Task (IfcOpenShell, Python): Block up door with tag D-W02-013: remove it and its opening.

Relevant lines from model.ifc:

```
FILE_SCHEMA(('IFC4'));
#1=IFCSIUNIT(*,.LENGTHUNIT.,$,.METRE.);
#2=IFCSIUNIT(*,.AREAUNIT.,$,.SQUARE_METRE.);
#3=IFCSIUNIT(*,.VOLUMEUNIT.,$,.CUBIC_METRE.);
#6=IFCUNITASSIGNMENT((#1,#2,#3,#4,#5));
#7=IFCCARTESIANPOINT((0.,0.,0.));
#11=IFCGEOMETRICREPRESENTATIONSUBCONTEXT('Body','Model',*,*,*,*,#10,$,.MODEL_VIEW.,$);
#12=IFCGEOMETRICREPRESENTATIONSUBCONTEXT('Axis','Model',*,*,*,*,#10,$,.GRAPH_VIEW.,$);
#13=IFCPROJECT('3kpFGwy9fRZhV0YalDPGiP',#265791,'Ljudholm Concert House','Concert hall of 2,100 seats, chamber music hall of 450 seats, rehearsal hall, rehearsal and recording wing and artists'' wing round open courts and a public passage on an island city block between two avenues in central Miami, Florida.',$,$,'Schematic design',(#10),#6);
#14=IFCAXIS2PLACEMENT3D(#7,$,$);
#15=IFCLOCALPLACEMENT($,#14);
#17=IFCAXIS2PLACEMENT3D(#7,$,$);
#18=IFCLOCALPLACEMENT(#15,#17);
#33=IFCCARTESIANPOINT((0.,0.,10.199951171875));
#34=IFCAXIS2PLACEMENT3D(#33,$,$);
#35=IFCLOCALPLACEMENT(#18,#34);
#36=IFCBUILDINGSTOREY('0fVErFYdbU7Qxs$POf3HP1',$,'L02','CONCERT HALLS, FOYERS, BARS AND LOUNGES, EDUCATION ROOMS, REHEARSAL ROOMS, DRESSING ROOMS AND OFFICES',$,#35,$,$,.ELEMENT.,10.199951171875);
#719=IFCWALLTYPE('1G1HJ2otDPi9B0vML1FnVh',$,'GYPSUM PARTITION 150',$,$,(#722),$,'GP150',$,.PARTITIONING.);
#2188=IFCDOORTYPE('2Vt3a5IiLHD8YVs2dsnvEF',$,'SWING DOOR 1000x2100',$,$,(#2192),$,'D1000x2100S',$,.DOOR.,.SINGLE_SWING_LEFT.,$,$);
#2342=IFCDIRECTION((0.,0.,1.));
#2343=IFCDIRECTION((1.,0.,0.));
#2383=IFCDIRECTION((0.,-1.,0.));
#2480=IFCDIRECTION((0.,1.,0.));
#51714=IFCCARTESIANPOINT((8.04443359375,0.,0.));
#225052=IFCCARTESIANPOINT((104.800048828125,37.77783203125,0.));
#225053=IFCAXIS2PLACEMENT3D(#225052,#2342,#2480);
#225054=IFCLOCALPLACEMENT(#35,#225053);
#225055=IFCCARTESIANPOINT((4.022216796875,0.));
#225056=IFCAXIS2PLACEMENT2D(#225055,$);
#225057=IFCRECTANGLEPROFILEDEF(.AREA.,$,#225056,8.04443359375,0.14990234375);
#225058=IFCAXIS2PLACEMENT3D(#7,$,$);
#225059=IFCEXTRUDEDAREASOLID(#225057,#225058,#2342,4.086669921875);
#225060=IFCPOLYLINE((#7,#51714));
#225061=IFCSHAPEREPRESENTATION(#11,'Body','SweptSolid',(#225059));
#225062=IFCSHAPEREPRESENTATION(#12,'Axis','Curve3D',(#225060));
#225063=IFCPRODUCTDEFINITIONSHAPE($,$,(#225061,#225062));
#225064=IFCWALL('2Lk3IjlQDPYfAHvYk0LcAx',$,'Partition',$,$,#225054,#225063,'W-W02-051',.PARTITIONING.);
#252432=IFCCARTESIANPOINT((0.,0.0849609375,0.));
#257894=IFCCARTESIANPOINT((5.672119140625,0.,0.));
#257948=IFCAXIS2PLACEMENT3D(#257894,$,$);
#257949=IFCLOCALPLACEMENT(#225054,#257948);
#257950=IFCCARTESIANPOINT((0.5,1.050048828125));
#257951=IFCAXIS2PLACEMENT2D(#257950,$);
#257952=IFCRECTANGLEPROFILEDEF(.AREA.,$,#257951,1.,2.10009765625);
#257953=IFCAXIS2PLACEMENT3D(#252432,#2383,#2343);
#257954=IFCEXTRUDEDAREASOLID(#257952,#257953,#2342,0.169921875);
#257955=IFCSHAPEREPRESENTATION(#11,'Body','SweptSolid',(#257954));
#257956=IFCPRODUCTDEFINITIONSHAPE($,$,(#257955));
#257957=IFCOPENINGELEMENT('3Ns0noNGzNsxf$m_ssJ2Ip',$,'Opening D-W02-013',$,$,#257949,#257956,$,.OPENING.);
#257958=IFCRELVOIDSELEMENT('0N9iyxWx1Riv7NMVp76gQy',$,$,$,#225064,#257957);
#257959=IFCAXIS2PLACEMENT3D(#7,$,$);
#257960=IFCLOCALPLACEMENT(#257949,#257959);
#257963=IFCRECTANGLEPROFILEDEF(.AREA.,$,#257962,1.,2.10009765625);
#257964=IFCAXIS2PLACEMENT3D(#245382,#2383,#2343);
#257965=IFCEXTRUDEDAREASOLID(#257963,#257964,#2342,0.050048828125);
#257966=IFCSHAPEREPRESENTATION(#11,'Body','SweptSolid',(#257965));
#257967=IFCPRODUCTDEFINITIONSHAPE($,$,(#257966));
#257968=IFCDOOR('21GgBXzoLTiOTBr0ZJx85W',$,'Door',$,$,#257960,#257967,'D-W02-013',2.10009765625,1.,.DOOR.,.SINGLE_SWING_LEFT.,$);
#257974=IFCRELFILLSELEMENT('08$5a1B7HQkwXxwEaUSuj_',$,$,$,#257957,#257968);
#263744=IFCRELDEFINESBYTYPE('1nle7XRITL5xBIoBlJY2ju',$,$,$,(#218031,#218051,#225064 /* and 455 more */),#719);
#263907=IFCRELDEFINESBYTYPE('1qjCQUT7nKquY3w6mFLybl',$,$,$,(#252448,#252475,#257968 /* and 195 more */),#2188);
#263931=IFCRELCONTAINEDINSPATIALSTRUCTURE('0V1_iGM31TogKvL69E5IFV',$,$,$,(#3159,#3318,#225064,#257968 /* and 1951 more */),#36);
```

```python
import ifcopenshell
import ifcopenshell.api.feature
import ifcopenshell.api.root
import ifcopenshell.geom
import ifcopenshell.util.shape

model = ifcopenshell.open("model.ifc")
settings = ifcopenshell.geom.settings()


def volume(element):
    """Net volume in cubic metres, openings subtracted."""
    shape = ifcopenshell.geom.create_shape(settings, element)
    return ifcopenshell.util.shape.get_volume(shape.geometry)


door = model.by_guid("21GgBXzoLTiOTBr0ZJx85W")
opening = door.FillsVoids[0].RelatingOpeningElement
wall = opening.VoidsElements[0].RelatingBuildingElement
before = volume(wall)

ifcopenshell.api.root.remove_product(model, product=door)
ifcopenshell.api.feature.remove_feature(model, feature=opening)

after = volume(wall)

print(f"wall volume {before:.3f} -> {after:.3f} m3")

model.write("model-out.ifc")
```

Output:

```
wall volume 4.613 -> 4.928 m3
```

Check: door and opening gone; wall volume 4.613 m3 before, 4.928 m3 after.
